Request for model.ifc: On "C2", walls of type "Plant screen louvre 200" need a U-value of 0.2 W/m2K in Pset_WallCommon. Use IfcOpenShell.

First a look at what the model holds.

```python
import ifcopenshell
import ifcopenshell.util.element

model = ifcopenshell.open("model.ifc")
print(model.schema)
storey = next(s for s in model.by_type("IfcBuildingStorey") if s.Name == "C2")
walls = [e for e in ifcopenshell.util.element.get_decomposition(storey) if e.is_a("IfcWall")]
seen = {}
for e in walls:
    element_type = ifcopenshell.util.element.get_type(e)
    key = (element_type.Name if element_type != e and element_type else None, ifcopenshell.util.element.get_pset(e, "Pset_WallCommon", "ThermalTransmittance"))
    seen[key] = seen.get(key, 0) + 1
for (name, value), count in sorted(seen.items(), key=str):
    print(count, "x", name, "|", value)
```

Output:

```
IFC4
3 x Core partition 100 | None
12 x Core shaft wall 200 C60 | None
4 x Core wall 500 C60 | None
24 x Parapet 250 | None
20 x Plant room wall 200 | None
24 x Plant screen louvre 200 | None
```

```python
import ifcopenshell
import ifcopenshell.api.pset
import ifcopenshell.util.element

model = ifcopenshell.open("model.ifc")

storey = next(s for s in model.by_type("IfcBuildingStorey") if s.Name == "C2")
walls = [e for e in ifcopenshell.util.element.get_decomposition(storey) if e.is_a("IfcWall")]

count = 0
for e in walls:
    element_type = ifcopenshell.util.element.get_type(e)
    if element_type in (None, e) or element_type.Name != "Plant screen louvre 200":
        continue
    found = ifcopenshell.util.element.get_pset(e, "Pset_WallCommon", should_inherit=False)
    if found:
        pset = model.by_id(found["id"])
        if len(ifcopenshell.util.element.get_elements_by_pset(pset)) > 1:
            pset = ifcopenshell.api.pset.unshare_pset(model, products=[e], pset=pset)[0]
    else:
        pset = ifcopenshell.api.pset.add_pset(model, product=e, name="Pset_WallCommon")
    ifcopenshell.api.pset.edit_pset(model, pset=pset, properties={"ThermalTransmittance": 0.2})
    count += 1

print(count, "walls updated")

model.write("model-out.ifc")
```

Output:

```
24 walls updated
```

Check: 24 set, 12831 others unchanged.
